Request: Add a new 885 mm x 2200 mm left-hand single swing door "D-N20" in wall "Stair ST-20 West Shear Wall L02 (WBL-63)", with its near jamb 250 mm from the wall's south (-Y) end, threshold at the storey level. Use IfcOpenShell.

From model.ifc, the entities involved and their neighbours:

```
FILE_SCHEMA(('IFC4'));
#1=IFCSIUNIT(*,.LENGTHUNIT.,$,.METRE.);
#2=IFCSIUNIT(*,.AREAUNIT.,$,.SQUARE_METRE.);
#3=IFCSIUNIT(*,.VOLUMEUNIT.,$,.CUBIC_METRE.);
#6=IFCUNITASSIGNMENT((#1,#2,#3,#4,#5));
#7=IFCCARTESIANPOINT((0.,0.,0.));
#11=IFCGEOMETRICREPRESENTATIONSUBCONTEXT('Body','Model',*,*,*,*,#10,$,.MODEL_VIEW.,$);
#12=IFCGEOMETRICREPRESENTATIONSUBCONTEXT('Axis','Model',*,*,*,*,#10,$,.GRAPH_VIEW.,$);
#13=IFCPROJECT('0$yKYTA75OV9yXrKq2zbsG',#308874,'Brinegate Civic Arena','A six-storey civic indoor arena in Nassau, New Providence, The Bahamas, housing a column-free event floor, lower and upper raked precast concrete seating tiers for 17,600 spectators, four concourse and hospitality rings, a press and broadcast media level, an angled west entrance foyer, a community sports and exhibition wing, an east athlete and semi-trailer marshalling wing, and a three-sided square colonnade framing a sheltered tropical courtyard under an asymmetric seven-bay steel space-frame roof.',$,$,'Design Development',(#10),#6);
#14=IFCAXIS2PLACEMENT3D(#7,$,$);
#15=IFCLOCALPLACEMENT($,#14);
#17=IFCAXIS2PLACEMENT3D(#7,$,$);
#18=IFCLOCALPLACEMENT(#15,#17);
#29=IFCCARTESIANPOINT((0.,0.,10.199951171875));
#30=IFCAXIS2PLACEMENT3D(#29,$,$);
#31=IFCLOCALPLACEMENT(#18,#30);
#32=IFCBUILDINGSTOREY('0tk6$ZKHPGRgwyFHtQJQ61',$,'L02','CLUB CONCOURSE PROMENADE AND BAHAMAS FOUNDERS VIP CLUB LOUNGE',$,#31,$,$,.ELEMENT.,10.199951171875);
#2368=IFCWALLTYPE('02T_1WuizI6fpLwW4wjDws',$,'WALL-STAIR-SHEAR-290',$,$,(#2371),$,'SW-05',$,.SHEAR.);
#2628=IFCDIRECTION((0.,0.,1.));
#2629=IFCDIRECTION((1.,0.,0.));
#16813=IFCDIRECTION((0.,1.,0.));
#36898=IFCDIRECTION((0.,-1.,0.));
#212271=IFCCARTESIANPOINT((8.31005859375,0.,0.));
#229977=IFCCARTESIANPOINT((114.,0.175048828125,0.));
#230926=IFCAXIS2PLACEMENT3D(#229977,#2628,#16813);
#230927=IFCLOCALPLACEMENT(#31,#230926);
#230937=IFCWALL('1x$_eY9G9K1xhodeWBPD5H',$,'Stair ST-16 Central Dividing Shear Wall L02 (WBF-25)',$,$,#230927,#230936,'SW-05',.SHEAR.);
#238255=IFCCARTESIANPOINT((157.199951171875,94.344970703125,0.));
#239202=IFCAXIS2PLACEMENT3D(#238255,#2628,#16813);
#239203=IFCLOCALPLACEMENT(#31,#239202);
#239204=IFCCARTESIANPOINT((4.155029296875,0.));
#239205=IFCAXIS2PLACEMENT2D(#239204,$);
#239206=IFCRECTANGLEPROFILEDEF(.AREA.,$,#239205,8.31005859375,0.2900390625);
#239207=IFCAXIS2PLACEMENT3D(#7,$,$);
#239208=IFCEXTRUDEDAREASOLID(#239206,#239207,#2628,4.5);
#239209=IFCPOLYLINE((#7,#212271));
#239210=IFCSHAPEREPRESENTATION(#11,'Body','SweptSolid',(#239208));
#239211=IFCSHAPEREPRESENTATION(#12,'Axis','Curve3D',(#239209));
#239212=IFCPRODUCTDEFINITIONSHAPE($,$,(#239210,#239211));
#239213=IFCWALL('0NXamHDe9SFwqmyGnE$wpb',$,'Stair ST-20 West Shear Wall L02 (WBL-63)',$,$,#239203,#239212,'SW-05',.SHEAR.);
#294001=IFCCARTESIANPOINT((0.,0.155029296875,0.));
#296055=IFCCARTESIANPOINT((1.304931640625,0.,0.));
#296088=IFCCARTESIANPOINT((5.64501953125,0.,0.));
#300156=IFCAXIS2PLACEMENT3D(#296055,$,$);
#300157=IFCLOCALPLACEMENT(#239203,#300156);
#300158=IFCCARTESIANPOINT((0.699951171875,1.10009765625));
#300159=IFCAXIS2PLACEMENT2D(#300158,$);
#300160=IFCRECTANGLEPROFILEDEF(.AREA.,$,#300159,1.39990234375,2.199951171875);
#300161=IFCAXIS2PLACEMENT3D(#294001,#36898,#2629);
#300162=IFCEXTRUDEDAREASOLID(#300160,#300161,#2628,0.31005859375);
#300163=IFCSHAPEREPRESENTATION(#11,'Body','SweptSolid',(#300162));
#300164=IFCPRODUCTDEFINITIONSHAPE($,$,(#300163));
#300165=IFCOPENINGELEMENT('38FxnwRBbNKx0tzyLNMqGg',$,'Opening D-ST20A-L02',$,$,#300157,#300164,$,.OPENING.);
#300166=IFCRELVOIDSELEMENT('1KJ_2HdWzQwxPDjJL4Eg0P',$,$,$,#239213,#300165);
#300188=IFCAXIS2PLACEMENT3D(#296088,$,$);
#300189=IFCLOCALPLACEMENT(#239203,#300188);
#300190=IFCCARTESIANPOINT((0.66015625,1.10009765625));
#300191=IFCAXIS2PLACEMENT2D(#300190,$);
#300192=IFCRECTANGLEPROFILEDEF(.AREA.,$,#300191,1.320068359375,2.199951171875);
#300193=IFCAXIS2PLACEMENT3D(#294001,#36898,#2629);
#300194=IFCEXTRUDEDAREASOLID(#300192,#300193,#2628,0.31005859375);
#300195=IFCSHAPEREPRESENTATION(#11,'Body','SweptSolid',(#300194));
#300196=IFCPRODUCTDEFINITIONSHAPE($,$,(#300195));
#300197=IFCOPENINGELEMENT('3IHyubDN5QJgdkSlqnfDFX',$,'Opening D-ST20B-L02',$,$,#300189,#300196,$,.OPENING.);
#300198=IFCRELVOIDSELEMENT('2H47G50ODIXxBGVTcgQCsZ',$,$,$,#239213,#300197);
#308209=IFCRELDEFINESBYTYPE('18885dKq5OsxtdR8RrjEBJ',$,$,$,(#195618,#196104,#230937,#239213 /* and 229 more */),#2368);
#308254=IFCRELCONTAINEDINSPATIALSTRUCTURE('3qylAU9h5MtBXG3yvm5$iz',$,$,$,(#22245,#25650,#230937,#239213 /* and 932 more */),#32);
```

```python
import numpy as np
import ifcopenshell
import ifcopenshell.api.feature
import ifcopenshell.api.geometry
import ifcopenshell.api.root
import ifcopenshell.api.spatial
import ifcopenshell.geom
import ifcopenshell.util.element
import ifcopenshell.util.placement
import ifcopenshell.util.representation
import ifcopenshell.util.shape
import ifcopenshell.util.unit

model = ifcopenshell.open("model.ifc")
unit_scale = ifcopenshell.util.unit.calculate_unit_scale(model)
settings = ifcopenshell.geom.settings()


def volume(element):
    """Net volume in cubic metres, openings subtracted."""
    shape = ifcopenshell.geom.create_shape(settings, element)
    return ifcopenshell.util.shape.get_volume(shape.geometry)


wall = model.by_guid("0NXamHDe9SFwqmyGnE$wpb")
storey = ifcopenshell.util.element.get_container(wall, ifc_class="IfcBuildingStorey")
context = ifcopenshell.util.representation.get_context(model, "Model", "Body", "MODEL_VIEW")
before = volume(wall)

width, height, from_end, sill = 0.885, 2.2, 0.25, 0.0  # metres

# The wall runs along its own X axis, and the end named is its -X end.
wall_shape = ifcopenshell.geom.create_shape(settings, wall)
x, y, z = ifcopenshell.util.shape.get_vertices(wall_shape.geometry).T
start = x.min() + from_end
face, thickness = float(y.min()), float(y.max() - y.min())
wall_matrix = ifcopenshell.util.placement.get_local_placement(wall.ObjectPlacement)
level = ifcopenshell.util.placement.get_local_placement(storey.ObjectPlacement)[2, 3]


def in_wall(x, y):
    """Placement at x, y metres in the wall's axes, at sill height."""
    matrix = wall_matrix.copy()
    matrix[:, 3] = wall_matrix @ np.array([x / unit_scale, y / unit_scale, 0.0, 1.0])
    matrix[2, 3] = level + sill / unit_scale
    return matrix


# Opening: a box that overshoots both wall faces by 50 mm.
opening = ifcopenshell.api.root.create_entity(model, ifc_class="IfcOpeningElement", predefined_type="OPENING")
box = ifcopenshell.api.geometry.add_wall_representation(
    model, context=context, length=width, height=height, thickness=thickness + 0.1
)
ifcopenshell.api.geometry.assign_representation(model, product=opening, representation=box)
ifcopenshell.api.geometry.edit_object_placement(model, product=opening, matrix=in_wall(start, face - 0.05), is_si=False)
ifcopenshell.api.feature.add_feature(model, feature=opening, element=wall)

door = ifcopenshell.api.root.create_entity(model, ifc_class="IfcDoor", name="D-N20", predefined_type="DOOR")
door.OverallWidth, door.OverallHeight = width / unit_scale, height / unit_scale
door.OperationType = "SINGLE_SWING_LEFT"
body = ifcopenshell.api.geometry.add_door_representation(
    model,
    context=context,
    overall_width=door.OverallWidth,
    overall_height=door.OverallHeight,
    operation_type="SINGLE_SWING_LEFT",
    lining_properties={"LiningDepth": thickness / unit_scale, "ThresholdDepth": thickness / unit_scale},
)
ifcopenshell.api.geometry.assign_representation(model, product=door, representation=body)
ifcopenshell.api.spatial.assign_container(model, products=[door], relating_structure=storey)
ifcopenshell.api.feature.add_filling(model, opening=opening, element=door)

# The lining spans the wall, so the door starts at the wall face.
ifcopenshell.api.geometry.edit_object_placement(model, product=door, matrix=in_wall(start, face), is_si=False)

after = volume(wall)

print(f"wall volume {before:.3f} -> {after:.3f} m3")

model.write("model_edited.ifc")
```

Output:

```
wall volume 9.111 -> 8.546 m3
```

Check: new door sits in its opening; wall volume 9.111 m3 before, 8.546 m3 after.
